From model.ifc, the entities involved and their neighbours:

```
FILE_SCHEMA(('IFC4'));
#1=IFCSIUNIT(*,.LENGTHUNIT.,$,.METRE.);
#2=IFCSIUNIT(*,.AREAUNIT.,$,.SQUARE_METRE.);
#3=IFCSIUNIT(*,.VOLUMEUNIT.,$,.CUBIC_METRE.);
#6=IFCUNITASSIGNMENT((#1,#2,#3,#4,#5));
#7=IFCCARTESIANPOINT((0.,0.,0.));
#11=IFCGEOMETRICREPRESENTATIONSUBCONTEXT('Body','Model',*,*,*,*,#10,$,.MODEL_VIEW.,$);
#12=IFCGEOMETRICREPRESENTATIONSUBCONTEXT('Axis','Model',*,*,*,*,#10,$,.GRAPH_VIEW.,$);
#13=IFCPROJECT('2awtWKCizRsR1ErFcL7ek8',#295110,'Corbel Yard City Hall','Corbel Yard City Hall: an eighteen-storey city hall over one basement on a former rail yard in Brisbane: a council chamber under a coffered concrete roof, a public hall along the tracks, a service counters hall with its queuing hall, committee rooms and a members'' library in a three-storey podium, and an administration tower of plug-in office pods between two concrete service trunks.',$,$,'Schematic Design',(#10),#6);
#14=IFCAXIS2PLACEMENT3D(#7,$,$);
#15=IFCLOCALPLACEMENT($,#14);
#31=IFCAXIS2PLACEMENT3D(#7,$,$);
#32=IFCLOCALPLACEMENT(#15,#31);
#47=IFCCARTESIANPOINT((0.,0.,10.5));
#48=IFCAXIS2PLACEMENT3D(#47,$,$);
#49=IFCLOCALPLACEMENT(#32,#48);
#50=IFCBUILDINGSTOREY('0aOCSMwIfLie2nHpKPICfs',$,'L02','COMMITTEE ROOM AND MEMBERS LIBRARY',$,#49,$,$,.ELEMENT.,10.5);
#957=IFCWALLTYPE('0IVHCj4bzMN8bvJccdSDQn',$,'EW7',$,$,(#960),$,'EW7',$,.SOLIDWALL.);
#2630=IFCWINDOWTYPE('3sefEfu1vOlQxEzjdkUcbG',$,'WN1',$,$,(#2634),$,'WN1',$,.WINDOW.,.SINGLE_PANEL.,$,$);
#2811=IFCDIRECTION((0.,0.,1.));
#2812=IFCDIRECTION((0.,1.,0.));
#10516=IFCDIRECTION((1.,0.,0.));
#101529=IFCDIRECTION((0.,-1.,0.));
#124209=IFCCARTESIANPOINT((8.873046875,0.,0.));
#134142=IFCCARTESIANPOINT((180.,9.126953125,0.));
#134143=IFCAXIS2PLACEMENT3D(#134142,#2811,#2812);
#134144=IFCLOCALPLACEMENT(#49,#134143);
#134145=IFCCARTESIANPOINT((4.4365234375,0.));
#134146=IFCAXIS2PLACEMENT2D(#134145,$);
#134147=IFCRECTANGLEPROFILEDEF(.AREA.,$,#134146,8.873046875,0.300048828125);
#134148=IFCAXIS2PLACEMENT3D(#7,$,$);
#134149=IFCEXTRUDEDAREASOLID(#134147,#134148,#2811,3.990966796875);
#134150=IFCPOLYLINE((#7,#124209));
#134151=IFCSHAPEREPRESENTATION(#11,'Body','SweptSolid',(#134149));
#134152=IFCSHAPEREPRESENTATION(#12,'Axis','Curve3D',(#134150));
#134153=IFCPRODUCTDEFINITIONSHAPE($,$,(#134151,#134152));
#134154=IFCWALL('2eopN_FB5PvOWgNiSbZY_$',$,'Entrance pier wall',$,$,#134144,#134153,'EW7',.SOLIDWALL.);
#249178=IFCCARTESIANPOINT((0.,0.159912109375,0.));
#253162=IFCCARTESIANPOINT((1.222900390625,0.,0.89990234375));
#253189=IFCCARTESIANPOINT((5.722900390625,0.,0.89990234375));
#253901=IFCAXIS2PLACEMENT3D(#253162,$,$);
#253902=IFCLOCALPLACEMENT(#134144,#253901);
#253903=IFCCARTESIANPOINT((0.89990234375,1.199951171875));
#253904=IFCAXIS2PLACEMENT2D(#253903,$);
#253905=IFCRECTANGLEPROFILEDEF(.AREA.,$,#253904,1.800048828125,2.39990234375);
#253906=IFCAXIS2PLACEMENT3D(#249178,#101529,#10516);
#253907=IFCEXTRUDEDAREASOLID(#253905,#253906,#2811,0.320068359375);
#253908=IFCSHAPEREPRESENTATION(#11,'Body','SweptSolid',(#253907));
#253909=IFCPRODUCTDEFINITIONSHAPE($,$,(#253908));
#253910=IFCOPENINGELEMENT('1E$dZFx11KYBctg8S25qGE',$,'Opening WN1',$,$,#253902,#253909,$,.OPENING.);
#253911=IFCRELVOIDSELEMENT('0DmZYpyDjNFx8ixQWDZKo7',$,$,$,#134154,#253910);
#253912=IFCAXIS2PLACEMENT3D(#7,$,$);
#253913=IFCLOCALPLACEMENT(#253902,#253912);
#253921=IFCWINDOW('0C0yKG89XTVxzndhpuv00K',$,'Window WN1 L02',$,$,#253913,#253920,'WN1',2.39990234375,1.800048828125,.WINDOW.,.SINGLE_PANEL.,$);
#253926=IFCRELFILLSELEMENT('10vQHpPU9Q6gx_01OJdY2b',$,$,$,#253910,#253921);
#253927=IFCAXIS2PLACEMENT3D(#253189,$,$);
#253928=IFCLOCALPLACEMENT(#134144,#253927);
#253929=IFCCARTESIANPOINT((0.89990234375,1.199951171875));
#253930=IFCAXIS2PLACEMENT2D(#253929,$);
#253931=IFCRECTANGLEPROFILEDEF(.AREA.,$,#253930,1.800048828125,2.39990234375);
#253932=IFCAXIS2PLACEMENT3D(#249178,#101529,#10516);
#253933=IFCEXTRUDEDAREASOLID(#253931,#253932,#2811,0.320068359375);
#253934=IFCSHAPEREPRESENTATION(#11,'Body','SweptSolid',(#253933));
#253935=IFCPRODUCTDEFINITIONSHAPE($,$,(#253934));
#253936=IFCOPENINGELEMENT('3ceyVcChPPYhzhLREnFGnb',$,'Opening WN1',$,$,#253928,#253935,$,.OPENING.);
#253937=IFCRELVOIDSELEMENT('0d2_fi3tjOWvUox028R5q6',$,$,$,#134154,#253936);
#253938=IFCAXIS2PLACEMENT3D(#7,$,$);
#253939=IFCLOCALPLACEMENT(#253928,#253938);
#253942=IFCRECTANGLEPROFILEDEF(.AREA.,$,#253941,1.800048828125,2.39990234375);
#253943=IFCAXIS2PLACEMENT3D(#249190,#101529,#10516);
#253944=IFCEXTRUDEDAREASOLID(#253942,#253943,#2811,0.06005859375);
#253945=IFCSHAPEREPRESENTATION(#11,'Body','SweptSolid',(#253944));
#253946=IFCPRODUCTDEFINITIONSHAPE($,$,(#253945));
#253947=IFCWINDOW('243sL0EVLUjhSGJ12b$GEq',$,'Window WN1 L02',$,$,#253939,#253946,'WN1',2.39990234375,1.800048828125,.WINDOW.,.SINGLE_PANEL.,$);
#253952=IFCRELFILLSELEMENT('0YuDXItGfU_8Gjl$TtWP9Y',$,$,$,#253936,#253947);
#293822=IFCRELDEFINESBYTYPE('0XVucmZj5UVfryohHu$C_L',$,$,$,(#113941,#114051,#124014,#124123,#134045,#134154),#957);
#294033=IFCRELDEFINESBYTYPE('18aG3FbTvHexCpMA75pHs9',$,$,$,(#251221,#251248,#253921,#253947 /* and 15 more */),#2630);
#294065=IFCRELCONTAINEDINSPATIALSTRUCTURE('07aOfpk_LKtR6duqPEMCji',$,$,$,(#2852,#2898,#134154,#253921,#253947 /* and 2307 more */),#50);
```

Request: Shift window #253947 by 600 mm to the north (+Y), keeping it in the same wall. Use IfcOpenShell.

```python
import ifcopenshell
import ifcopenshell.api.geometry
import ifcopenshell.util.placement

model = ifcopenshell.open("model.ifc")

window = model.by_guid("243sL0EVLUjhSGJ12b$GEq")
opening = window.FillsVoids[0].RelatingOpeningElement
wall = opening.VoidsElements[0].RelatingBuildingElement

wall_matrix = ifcopenshell.util.placement.get_local_placement(wall.ObjectPlacement)
shift = wall_matrix[:3, 0] * 0.6
before = ifcopenshell.util.placement.get_local_placement(window.ObjectPlacement)[:3, 3].copy()

# The window is placed relative to its opening, so it follows when the opening moves.
matrix = ifcopenshell.util.placement.get_local_placement(opening.ObjectPlacement)
matrix[:3, 3] += shift
ifcopenshell.api.geometry.edit_object_placement(
    model, product=opening, matrix=matrix, is_si=False, should_transform_children=True
)

after = ifcopenshell.util.placement.get_local_placement(window.ObjectPlacement)[:3, 3]
print("window moved by", (after - before).round(3) + 0.0)

model.write("model_updated.ifc")
```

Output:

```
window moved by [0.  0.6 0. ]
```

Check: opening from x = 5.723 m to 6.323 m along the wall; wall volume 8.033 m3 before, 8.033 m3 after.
